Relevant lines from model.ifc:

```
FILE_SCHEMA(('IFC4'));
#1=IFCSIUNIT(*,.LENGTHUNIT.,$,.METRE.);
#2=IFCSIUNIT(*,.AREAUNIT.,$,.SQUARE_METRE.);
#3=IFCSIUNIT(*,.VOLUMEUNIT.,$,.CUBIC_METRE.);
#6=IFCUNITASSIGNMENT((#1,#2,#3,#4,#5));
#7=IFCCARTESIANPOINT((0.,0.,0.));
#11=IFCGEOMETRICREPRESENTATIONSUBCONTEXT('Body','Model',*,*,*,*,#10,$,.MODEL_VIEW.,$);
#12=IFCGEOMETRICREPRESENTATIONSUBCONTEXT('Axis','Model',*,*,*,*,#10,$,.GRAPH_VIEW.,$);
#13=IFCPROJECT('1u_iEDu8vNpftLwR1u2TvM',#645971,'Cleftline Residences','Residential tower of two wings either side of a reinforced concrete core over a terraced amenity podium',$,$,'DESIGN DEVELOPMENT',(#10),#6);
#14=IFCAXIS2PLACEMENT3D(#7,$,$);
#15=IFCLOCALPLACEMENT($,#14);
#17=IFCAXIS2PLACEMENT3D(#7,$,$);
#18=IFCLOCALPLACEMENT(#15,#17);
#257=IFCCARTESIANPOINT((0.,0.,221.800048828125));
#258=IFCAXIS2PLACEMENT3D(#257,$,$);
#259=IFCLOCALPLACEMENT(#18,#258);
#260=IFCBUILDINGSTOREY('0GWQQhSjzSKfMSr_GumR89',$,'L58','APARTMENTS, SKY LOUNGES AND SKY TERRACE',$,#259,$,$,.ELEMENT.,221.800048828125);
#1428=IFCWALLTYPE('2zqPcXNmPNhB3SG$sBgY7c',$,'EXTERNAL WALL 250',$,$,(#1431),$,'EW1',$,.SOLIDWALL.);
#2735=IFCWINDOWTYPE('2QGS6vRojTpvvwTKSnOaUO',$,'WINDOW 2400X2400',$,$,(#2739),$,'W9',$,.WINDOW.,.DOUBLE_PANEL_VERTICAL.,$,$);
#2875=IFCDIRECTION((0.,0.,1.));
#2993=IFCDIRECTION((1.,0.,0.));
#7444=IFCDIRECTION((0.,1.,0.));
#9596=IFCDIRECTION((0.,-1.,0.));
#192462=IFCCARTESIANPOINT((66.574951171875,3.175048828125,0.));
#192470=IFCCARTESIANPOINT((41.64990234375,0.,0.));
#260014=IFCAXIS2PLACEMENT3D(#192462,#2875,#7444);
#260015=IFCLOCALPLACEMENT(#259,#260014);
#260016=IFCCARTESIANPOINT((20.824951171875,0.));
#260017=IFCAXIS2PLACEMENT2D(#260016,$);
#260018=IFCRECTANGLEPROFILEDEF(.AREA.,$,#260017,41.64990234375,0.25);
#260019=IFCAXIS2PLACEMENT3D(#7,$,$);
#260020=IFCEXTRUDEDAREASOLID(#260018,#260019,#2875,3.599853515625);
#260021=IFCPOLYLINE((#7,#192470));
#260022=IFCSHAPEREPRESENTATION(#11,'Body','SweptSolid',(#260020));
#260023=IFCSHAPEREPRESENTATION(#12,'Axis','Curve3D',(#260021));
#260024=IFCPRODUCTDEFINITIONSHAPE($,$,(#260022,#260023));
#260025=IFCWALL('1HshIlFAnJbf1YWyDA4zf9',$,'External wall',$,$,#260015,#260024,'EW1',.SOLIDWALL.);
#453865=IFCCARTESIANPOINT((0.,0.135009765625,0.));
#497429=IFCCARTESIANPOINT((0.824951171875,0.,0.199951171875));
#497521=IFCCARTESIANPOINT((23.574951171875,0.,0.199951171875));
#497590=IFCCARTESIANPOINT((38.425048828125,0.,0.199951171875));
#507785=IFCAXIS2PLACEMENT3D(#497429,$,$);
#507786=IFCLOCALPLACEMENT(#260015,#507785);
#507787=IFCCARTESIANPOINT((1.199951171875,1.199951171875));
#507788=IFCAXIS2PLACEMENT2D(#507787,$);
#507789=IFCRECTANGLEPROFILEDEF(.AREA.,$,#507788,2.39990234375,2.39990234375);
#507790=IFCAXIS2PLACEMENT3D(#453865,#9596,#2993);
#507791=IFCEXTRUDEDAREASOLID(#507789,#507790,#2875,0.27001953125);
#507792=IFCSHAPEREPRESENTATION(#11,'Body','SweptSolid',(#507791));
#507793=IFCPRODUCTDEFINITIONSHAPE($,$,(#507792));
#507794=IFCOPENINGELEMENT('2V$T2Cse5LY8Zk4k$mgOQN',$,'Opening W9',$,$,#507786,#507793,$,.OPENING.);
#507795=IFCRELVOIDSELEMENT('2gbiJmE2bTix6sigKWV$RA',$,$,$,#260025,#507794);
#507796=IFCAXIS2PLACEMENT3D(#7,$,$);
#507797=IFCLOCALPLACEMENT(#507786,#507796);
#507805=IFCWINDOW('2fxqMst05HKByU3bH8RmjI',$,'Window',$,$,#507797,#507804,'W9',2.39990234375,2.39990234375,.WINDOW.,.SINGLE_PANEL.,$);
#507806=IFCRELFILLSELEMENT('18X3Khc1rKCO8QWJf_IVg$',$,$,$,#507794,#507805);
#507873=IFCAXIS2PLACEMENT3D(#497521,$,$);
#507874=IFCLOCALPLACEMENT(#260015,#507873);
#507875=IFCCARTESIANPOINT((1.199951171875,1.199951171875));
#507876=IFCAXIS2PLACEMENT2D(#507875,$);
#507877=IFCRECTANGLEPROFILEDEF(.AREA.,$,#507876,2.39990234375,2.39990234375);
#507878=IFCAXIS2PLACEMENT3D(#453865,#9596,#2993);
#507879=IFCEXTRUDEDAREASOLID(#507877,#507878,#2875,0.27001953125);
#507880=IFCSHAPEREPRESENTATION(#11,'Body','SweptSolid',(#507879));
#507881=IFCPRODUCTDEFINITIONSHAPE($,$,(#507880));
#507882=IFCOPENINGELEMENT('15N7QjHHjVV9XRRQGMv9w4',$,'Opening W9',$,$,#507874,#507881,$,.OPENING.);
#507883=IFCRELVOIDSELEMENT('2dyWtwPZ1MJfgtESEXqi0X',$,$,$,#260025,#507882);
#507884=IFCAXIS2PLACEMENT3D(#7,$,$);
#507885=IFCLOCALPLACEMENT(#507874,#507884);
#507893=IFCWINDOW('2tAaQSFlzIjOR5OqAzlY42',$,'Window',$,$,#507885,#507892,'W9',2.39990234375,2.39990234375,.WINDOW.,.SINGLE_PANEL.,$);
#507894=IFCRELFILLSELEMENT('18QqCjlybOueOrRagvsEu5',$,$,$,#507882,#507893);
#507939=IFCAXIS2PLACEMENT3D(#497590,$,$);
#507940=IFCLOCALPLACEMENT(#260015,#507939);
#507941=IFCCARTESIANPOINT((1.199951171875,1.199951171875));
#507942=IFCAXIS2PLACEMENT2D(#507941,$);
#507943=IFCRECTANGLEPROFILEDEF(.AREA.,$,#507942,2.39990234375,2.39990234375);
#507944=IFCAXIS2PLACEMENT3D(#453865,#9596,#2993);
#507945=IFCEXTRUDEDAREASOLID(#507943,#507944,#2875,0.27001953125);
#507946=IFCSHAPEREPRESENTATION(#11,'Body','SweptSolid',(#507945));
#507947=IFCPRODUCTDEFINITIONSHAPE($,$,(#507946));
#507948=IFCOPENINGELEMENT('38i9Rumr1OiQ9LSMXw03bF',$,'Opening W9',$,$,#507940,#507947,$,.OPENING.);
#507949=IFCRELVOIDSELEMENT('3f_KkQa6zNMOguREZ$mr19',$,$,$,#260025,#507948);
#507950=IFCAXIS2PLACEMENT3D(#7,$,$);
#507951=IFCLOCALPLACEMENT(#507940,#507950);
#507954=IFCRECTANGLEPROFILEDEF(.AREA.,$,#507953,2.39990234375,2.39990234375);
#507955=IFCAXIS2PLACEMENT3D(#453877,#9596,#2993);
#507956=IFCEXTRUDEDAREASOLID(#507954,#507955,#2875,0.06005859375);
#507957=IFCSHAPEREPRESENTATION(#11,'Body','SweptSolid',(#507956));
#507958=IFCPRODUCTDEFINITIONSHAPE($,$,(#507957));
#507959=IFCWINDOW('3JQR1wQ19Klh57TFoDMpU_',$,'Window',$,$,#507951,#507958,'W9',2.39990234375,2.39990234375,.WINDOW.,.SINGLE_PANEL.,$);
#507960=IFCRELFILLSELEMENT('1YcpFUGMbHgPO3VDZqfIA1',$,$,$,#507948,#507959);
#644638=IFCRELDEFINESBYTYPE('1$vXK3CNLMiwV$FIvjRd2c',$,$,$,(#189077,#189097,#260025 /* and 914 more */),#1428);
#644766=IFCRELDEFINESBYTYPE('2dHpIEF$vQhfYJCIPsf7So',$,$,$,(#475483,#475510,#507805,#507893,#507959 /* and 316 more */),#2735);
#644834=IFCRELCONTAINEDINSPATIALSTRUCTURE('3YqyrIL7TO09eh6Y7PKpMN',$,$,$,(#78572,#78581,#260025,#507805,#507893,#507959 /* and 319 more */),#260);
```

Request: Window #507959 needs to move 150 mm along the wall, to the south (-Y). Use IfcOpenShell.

```python
import ifcopenshell
import ifcopenshell.api.geometry
import ifcopenshell.util.placement
import ifcopenshell.util.unit

model = ifcopenshell.open("model.ifc")
unit_scale = ifcopenshell.util.unit.calculate_unit_scale(model)

window = model.by_id(507959)
opening = window.FillsVoids[0].RelatingOpeningElement
wall = opening.VoidsElements[0].RelatingBuildingElement

wall_matrix = ifcopenshell.util.placement.get_local_placement(wall.ObjectPlacement)
shift = wall_matrix[:3, 0] * -0.15 / unit_scale
before = ifcopenshell.util.placement.get_local_placement(window.ObjectPlacement)[:3, 3].copy()

# The window is placed relative to its opening, so it follows when the opening moves.
matrix = ifcopenshell.util.placement.get_local_placement(opening.ObjectPlacement)
matrix[:3, 3] += shift
ifcopenshell.api.geometry.edit_object_placement(
    model, product=opening, matrix=matrix, is_si=False, should_transform_children=True
)

after = ifcopenshell.util.placement.get_local_placement(window.ObjectPlacement)[:3, 3]
print("window moved by", (after - before).round(3) + 0.0)

model.write("model_edited.ifc")
```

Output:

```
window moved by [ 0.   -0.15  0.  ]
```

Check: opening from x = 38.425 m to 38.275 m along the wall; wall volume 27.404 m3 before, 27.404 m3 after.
